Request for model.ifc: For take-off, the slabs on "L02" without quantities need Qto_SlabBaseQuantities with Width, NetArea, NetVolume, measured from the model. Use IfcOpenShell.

First a look at what the model holds.

```python
import ifcopenshell
import ifcopenshell.util.element
import ifcopenshell.util.unit

model = ifcopenshell.open("model.ifc")
print(model.schema)
for unit_type in ("LENGTHUNIT", "AREAUNIT", "VOLUMEUNIT"):
    print(unit_type, ifcopenshell.util.unit.calculate_unit_scale(model, unit_type))
storey = next(s for s in model.by_type("IfcBuildingStorey") if s.Name == "L02")
slabs = [e for e in ifcopenshell.util.element.get_decomposition(storey) if e.is_a("IfcSlab")]
for e in sorted(slabs, key=lambda e: e.id()):
    print(e.id(), e.is_a(), e.Name, list(ifcopenshell.util.element.get_psets(e, qtos_only=True)), sep=" | ")
```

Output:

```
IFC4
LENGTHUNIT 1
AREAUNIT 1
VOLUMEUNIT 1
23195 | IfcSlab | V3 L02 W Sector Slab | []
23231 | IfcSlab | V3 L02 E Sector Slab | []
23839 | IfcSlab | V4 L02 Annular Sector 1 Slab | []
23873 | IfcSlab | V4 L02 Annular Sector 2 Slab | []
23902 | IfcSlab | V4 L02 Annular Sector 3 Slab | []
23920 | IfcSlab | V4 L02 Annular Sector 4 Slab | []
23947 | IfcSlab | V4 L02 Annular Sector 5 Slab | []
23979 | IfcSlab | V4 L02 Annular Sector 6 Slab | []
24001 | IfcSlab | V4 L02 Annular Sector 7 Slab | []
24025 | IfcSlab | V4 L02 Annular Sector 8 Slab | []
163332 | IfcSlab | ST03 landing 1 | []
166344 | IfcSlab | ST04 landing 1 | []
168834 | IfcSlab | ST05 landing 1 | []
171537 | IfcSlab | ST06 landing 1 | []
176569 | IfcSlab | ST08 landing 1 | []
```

```python
import ifcopenshell
import ifcopenshell.api.pset
import ifcopenshell.geom
import ifcopenshell.util.element
import ifcopenshell.util.shape
import ifcopenshell.util.unit

model = ifcopenshell.open("model.ifc")
unit_scale = ifcopenshell.util.unit.calculate_unit_scale(model)
area_scale = ifcopenshell.util.unit.calculate_unit_scale(model, "AREAUNIT")
volume_scale = ifcopenshell.util.unit.calculate_unit_scale(model, "VOLUMEUNIT")
settings = ifcopenshell.geom.settings()

storey = next(s for s in model.by_type("IfcBuildingStorey") if s.Name == "L02")
slabs = [e for e in ifcopenshell.util.element.get_decomposition(storey) if e.is_a("IfcSlab")]

for e in sorted(slabs, key=lambda e: e.id()):
    if ifcopenshell.util.element.get_psets(e, qtos_only=True, should_inherit=False):
        continue
    # Geometry comes back in metres, in the element's own axes.
    shape = ifcopenshell.geom.create_shape(settings, e)
    values = {
        "Width": ifcopenshell.util.shape.get_z(shape.geometry) / unit_scale,
        "NetArea": ifcopenshell.util.shape.get_footprint_area(shape.geometry) / area_scale,
        "NetVolume": ifcopenshell.util.shape.get_volume(shape.geometry) / volume_scale,
    }
    qto = ifcopenshell.api.pset.add_qto(model, product=e, name="Qto_SlabBaseQuantities")
    ifcopenshell.api.pset.edit_qto(model, qto=qto, properties=values)
    print(e.id(), {k: round(v, 3) for k, v in values.items()})

model.write("model-out.ifc")
```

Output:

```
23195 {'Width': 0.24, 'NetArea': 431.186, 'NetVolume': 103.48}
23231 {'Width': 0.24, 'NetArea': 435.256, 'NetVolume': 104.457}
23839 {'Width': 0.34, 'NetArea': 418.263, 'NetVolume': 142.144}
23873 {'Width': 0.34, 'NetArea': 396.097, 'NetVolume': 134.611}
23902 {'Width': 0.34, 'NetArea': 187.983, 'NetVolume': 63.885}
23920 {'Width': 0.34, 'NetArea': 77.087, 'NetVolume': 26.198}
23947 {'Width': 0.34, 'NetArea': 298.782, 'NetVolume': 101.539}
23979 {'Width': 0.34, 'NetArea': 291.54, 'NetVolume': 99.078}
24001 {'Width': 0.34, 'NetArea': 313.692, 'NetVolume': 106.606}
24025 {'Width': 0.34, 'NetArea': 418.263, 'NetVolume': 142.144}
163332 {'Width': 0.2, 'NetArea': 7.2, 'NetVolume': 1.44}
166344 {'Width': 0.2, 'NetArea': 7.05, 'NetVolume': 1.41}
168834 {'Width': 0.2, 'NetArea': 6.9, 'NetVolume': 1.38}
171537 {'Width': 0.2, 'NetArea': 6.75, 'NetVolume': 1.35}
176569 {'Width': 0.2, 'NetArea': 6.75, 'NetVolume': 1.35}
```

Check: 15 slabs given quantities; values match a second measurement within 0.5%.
